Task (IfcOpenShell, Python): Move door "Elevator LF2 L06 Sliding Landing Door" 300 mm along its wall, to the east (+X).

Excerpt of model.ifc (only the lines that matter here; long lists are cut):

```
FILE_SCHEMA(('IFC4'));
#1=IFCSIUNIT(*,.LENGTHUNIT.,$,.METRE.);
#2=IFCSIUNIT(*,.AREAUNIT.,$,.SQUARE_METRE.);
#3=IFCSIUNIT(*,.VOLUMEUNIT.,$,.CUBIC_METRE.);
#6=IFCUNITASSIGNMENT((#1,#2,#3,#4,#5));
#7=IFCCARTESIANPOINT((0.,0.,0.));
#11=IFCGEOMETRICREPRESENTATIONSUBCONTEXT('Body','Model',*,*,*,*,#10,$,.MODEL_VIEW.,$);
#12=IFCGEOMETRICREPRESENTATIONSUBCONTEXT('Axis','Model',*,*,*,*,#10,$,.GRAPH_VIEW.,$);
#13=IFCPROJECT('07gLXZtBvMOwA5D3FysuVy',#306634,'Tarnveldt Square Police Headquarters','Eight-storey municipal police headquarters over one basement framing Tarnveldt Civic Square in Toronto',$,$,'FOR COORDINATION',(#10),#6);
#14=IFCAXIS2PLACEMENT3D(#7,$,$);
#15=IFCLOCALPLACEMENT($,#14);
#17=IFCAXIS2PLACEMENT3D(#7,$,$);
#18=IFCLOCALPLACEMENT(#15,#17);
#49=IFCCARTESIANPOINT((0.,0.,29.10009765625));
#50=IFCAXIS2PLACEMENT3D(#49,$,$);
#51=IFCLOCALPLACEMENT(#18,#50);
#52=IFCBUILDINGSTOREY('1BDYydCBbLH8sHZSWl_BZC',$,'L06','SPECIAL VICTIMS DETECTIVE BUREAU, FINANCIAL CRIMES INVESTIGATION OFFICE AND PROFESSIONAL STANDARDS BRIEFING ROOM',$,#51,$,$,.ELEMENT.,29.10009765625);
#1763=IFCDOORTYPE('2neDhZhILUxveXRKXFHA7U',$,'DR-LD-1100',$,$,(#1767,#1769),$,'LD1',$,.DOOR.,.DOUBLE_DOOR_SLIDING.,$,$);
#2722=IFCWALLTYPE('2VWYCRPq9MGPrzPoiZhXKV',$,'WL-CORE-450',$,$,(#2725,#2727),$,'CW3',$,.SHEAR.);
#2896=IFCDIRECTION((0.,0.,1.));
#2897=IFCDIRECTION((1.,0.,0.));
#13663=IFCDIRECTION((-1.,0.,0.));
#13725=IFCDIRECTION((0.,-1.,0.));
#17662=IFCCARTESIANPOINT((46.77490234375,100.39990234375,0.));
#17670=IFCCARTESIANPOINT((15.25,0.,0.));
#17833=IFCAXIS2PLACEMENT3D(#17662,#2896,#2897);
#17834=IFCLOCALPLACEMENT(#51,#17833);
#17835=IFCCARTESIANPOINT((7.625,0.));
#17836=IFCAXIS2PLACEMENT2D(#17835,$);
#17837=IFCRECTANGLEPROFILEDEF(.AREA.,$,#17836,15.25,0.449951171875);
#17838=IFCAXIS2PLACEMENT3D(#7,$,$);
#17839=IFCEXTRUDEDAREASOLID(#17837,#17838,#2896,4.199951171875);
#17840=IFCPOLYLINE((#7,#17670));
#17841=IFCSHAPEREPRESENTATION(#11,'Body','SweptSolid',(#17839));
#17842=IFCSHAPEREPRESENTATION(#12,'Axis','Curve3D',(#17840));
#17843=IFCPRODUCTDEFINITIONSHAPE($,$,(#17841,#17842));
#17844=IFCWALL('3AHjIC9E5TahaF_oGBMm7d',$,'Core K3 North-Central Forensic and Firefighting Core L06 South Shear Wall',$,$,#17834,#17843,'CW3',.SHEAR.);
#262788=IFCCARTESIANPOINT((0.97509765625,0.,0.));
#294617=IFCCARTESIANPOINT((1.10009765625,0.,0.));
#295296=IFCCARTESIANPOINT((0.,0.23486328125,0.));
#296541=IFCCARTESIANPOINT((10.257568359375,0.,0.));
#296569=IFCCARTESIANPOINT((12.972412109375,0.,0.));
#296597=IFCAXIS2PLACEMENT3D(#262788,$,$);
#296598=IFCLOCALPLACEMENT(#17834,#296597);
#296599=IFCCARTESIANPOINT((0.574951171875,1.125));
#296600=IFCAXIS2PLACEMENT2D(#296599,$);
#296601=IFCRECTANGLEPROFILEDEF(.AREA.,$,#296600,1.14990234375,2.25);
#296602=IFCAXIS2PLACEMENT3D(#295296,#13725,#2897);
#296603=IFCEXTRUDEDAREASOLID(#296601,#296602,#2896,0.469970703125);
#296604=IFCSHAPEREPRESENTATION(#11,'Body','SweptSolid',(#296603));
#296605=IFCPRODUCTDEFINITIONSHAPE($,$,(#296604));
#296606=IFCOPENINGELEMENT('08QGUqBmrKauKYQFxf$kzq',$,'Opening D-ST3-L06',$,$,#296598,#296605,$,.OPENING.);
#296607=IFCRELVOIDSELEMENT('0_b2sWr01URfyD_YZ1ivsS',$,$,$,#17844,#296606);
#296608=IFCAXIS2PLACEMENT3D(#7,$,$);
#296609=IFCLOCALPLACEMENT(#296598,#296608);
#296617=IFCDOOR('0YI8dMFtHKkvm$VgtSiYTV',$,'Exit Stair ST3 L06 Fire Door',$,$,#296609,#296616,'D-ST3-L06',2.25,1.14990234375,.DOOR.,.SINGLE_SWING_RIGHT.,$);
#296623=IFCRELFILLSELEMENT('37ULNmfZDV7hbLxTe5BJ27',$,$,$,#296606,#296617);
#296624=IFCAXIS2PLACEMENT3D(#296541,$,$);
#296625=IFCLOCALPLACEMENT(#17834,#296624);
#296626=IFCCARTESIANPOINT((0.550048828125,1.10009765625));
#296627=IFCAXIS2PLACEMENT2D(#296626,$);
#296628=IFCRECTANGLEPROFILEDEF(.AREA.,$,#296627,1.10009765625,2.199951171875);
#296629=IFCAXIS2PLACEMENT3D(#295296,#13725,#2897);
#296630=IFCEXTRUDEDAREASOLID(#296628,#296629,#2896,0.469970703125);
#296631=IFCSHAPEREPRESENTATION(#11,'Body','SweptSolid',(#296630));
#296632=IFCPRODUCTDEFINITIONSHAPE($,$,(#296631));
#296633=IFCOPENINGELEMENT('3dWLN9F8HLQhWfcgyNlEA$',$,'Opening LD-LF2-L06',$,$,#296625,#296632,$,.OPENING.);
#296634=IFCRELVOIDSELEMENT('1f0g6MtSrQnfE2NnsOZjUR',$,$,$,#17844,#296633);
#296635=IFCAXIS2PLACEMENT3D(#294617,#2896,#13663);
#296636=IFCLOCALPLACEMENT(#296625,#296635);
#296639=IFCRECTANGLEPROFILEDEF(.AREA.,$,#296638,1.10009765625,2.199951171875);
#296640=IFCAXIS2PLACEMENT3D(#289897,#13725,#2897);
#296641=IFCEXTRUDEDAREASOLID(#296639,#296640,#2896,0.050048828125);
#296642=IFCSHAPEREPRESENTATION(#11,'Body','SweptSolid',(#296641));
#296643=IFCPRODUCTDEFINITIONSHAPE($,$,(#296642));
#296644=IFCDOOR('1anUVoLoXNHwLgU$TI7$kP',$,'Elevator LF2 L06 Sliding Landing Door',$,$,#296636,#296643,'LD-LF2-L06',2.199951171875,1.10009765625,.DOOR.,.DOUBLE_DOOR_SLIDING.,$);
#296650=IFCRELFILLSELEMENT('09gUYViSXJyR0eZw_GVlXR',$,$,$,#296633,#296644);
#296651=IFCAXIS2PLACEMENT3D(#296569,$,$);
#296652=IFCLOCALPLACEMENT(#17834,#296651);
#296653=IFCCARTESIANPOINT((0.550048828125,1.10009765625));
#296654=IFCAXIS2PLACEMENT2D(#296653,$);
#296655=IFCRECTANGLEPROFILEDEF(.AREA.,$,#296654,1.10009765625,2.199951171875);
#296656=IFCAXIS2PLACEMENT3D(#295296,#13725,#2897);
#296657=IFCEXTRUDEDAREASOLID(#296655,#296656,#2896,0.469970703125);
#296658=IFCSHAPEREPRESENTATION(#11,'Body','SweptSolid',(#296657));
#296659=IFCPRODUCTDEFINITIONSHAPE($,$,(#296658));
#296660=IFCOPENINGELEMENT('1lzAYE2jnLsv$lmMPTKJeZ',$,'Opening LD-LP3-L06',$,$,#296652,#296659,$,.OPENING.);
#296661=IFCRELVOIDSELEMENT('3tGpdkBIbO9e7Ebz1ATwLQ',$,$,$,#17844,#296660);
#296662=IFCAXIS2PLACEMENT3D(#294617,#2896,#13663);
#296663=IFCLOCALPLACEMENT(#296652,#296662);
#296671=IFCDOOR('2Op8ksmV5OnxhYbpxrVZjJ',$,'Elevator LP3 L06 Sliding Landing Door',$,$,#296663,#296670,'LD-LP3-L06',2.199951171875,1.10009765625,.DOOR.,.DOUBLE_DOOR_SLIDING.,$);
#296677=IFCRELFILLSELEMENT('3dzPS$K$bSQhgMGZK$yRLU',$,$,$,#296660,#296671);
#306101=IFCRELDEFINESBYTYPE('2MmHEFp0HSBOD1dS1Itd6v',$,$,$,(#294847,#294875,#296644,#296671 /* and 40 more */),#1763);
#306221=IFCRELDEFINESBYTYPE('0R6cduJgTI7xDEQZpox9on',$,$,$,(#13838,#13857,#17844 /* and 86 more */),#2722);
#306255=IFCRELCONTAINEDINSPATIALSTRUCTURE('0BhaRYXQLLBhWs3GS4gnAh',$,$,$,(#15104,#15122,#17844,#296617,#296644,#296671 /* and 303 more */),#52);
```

```python
import ifcopenshell
import ifcopenshell.api.geometry
import ifcopenshell.util.placement
import ifcopenshell.util.unit

model = ifcopenshell.open("model.ifc")
unit_scale = ifcopenshell.util.unit.calculate_unit_scale(model)

door = model.by_guid("1anUVoLoXNHwLgU$TI7$kP")
opening = door.FillsVoids[0].RelatingOpeningElement
wall = opening.VoidsElements[0].RelatingBuildingElement

wall_matrix = ifcopenshell.util.placement.get_local_placement(wall.ObjectPlacement)
shift = wall_matrix[:3, 0] * 0.3 / unit_scale
before = ifcopenshell.util.placement.get_local_placement(door.ObjectPlacement)[:3, 3].copy()

# The door is placed relative to its opening, so it follows when the opening moves.
matrix = ifcopenshell.util.placement.get_local_placement(opening.ObjectPlacement)
matrix[:3, 3] += shift
ifcopenshell.api.geometry.edit_object_placement(
    model, product=opening, matrix=matrix, is_si=False, should_transform_children=True
)

after = ifcopenshell.util.placement.get_local_placement(door.ObjectPlacement)[:3, 3]
print("door moved by", (after - before).round(3) + 0.0)

model.write("model-out.ifc")
```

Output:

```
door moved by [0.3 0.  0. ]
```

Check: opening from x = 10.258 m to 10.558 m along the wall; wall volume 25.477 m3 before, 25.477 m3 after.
